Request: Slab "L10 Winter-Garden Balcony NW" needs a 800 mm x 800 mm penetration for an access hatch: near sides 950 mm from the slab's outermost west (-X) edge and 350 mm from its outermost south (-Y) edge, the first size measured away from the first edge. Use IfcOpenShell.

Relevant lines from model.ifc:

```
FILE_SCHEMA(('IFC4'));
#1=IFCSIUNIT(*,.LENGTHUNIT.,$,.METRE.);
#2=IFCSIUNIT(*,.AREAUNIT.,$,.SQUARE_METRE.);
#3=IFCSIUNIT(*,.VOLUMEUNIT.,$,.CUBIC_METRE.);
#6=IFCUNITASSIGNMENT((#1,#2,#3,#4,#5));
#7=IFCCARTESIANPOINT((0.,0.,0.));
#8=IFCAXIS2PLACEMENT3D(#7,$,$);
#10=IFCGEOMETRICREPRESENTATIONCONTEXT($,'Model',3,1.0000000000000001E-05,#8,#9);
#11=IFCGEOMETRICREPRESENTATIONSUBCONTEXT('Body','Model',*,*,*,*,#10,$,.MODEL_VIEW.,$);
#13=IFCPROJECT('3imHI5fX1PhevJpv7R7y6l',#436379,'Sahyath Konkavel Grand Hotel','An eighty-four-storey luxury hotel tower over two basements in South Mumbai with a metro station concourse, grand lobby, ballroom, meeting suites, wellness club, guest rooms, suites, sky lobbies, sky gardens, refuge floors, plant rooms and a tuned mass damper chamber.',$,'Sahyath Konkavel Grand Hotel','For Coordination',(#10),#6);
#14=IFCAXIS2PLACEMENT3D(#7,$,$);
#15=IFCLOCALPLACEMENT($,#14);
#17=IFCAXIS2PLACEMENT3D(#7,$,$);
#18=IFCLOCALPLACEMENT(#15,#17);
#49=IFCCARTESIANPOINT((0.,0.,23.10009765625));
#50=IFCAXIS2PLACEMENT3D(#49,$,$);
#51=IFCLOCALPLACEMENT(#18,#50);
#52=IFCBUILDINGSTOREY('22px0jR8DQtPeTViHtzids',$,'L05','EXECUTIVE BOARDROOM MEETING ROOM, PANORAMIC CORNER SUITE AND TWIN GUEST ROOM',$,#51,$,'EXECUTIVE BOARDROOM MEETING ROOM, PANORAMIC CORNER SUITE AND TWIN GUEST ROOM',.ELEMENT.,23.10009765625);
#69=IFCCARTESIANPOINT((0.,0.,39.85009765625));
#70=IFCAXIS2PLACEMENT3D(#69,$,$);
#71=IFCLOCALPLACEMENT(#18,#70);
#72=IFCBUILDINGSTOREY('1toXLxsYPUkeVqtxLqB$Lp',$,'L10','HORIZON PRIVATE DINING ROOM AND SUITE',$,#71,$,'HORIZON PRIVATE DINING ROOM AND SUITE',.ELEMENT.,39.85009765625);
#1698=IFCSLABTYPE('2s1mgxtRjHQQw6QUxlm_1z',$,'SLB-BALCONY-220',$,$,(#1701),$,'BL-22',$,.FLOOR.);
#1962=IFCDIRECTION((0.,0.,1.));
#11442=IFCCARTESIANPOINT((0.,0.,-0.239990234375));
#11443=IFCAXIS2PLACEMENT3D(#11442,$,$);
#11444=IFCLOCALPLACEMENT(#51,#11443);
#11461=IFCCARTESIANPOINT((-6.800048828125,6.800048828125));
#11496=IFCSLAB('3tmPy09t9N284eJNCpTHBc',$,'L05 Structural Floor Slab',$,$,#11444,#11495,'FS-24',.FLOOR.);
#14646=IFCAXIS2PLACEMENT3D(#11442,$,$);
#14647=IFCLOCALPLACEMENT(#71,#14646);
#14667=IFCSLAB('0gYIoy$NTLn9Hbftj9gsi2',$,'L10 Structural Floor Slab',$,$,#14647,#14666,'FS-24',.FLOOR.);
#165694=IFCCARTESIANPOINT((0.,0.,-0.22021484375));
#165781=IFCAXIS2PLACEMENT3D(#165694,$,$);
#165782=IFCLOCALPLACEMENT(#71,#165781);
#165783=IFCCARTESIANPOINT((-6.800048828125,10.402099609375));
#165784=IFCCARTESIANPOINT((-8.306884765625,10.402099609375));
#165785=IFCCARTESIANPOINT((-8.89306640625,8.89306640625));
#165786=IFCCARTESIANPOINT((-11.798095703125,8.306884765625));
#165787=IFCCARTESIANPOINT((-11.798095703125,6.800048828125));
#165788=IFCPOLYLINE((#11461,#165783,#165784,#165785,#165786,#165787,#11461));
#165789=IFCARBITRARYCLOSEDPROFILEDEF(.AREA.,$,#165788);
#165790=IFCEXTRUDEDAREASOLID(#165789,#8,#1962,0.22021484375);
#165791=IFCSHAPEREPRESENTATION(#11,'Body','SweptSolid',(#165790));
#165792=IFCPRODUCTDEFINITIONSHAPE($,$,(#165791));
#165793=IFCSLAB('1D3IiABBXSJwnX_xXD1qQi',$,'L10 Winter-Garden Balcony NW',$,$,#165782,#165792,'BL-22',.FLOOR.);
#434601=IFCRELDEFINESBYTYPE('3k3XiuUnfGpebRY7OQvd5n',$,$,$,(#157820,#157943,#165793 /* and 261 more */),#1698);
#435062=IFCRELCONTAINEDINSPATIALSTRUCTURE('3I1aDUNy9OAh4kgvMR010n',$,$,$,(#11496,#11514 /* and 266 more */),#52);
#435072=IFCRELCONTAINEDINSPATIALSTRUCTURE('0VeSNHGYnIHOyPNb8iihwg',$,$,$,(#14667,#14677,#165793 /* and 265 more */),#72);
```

```python
import numpy as np
import ifcopenshell
import ifcopenshell.api.feature
import ifcopenshell.api.geometry
import ifcopenshell.api.root
import ifcopenshell.geom
import ifcopenshell.util.placement
import ifcopenshell.util.representation
import ifcopenshell.util.shape
import ifcopenshell.util.unit

model = ifcopenshell.open("model.ifc")
unit_scale = ifcopenshell.util.unit.calculate_unit_scale(model)
settings = ifcopenshell.geom.settings()


def volume(element):
    """Net volume in cubic metres, openings subtracted."""
    shape = ifcopenshell.geom.create_shape(settings, element)
    return ifcopenshell.util.shape.get_volume(shape.geometry)


slab = model.by_guid("1D3IiABBXSJwnX_xXD1qQi")
before = volume(slab)

# Extent in the slab's own axes, in metres. The edges named are its -X and -Y sides.
slab_shape = ifcopenshell.geom.create_shape(settings, slab)
vertices = ifcopenshell.util.shape.get_vertices(slab_shape.geometry)
x_min, y_min, bottom = vertices.min(axis=0)
top = vertices[:, 2].max()

opening = ifcopenshell.api.root.create_entity(model, ifc_class="IfcOpeningElement", name="Access hatch opening", predefined_type="OPENING")
context = ifcopenshell.util.representation.get_context(model, "Model", "Body", "MODEL_VIEW")
width, depth = 0.8, 0.8
outline = [(0.0, 0.0), (width, 0.0), (width, depth), (0.0, depth), (0.0, 0.0)]
# Overshoot both faces by 50 mm so the cut is clean.
shape = ifcopenshell.api.geometry.add_slab_representation(
    model, context=context, depth=top - bottom + 0.1, polyline=outline
)
ifcopenshell.api.geometry.assign_representation(model, product=opening, representation=shape)

matrix = ifcopenshell.util.placement.get_local_placement(slab.ObjectPlacement)
matrix[:, 3] = matrix @ np.append(np.array([x_min + 0.95, y_min + 0.35, bottom - 0.05]) / unit_scale, 1.0)
ifcopenshell.api.geometry.edit_object_placement(model, product=opening, matrix=matrix, is_si=False)
ifcopenshell.api.feature.add_feature(model, feature=opening, element=slab)

after = volume(slab)

print(f"slab volume {before:.3f} -> {after:.3f} m3")

model.write("model_rev.ifc")
```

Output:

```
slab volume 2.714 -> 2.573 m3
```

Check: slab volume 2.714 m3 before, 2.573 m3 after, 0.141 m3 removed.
